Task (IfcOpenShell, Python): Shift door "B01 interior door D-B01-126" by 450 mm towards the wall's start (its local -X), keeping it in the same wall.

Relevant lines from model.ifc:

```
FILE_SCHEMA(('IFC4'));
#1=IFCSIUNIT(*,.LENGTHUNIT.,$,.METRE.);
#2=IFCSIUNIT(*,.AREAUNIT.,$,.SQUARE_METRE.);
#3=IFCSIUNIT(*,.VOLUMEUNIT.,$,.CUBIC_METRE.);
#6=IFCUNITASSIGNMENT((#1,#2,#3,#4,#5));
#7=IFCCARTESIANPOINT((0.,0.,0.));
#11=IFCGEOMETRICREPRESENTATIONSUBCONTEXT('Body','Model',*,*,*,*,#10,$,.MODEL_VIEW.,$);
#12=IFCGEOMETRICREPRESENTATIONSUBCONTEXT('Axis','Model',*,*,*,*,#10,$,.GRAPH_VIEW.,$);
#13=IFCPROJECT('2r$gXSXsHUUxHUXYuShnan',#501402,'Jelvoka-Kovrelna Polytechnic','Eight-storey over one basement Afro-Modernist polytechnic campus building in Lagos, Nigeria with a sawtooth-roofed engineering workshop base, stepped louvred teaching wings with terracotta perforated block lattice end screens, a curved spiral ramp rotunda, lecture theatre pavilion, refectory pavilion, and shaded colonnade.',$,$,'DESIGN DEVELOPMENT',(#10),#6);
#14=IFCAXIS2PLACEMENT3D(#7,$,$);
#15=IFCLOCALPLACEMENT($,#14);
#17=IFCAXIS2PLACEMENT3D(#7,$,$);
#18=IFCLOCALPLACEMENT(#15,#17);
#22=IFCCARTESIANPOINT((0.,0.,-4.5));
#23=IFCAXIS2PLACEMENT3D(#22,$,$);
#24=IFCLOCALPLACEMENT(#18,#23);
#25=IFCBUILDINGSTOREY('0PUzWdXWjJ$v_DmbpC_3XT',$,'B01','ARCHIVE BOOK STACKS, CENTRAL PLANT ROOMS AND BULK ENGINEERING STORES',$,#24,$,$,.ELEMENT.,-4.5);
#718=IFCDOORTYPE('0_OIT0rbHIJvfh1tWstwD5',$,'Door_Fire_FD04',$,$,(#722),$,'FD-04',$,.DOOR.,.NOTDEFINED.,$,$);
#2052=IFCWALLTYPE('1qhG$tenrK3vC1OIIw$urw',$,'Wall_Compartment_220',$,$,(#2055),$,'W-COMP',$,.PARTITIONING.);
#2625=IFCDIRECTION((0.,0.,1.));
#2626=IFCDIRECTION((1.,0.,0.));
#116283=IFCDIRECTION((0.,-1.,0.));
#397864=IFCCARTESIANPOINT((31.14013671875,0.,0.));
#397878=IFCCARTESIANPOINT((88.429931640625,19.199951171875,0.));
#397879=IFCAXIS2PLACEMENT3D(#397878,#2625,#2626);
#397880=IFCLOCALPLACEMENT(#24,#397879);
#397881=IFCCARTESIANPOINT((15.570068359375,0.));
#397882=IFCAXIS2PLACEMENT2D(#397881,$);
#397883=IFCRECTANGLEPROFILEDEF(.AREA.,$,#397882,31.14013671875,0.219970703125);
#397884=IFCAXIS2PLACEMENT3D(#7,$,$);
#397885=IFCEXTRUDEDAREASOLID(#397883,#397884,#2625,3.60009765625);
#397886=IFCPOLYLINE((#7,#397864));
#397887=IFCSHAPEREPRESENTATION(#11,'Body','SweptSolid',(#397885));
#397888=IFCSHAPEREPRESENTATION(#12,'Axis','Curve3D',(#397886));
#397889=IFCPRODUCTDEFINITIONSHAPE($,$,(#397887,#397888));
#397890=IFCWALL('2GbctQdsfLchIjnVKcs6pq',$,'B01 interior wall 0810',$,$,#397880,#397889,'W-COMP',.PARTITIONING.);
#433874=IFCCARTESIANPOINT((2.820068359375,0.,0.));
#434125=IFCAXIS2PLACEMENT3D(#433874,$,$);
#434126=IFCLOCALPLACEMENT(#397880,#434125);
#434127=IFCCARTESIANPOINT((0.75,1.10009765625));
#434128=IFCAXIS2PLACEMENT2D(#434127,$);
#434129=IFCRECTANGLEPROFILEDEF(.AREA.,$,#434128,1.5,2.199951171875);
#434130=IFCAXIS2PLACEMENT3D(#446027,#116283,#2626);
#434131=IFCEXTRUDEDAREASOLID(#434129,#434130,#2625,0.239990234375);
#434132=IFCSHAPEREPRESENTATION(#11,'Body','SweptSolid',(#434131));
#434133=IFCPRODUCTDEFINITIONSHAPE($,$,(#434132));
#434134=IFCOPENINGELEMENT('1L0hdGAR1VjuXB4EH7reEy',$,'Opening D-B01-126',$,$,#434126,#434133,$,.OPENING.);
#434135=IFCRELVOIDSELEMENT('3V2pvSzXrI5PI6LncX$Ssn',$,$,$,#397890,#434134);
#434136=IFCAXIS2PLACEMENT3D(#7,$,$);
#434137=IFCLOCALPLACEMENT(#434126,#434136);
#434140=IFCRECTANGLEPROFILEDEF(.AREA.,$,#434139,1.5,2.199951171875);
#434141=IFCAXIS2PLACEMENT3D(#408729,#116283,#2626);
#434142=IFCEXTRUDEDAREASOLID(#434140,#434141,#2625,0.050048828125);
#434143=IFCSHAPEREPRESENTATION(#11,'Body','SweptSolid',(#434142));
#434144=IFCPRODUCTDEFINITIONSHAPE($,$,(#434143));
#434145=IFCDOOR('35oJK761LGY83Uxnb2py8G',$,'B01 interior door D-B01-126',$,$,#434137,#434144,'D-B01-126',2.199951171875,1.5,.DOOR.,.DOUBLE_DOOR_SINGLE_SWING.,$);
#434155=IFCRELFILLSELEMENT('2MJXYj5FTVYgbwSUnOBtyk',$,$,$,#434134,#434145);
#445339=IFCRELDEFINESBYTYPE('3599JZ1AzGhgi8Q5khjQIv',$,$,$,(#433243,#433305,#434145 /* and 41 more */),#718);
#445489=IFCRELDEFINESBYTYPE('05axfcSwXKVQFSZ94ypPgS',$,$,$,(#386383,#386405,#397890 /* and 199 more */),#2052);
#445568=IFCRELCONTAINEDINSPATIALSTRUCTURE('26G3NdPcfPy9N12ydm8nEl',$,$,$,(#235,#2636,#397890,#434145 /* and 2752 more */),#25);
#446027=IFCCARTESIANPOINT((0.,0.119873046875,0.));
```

```python
import ifcopenshell
import ifcopenshell.api.geometry
import ifcopenshell.util.placement
import ifcopenshell.util.unit

model = ifcopenshell.open("model.ifc")
unit_scale = ifcopenshell.util.unit.calculate_unit_scale(model)

door = model.by_guid("35oJK761LGY83Uxnb2py8G")
opening = door.FillsVoids[0].RelatingOpeningElement
wall = opening.VoidsElements[0].RelatingBuildingElement

wall_matrix = ifcopenshell.util.placement.get_local_placement(wall.ObjectPlacement)
shift = wall_matrix[:3, 0] * -0.45 / unit_scale
before = ifcopenshell.util.placement.get_local_placement(door.ObjectPlacement)[:3, 3].copy()

# The door is placed relative to its opening, so it follows when the opening moves.
matrix = ifcopenshell.util.placement.get_local_placement(opening.ObjectPlacement)
matrix[:3, 3] += shift
ifcopenshell.api.geometry.edit_object_placement(
    model, product=opening, matrix=matrix, is_si=False, should_transform_children=True
)

after = ifcopenshell.util.placement.get_local_placement(door.ObjectPlacement)[:3, 3]
print("door moved by", (after - before).round(3) + 0.0)

model.write("model_rev.ifc")
```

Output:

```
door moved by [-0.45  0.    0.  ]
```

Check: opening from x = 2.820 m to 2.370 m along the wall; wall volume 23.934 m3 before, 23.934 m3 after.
